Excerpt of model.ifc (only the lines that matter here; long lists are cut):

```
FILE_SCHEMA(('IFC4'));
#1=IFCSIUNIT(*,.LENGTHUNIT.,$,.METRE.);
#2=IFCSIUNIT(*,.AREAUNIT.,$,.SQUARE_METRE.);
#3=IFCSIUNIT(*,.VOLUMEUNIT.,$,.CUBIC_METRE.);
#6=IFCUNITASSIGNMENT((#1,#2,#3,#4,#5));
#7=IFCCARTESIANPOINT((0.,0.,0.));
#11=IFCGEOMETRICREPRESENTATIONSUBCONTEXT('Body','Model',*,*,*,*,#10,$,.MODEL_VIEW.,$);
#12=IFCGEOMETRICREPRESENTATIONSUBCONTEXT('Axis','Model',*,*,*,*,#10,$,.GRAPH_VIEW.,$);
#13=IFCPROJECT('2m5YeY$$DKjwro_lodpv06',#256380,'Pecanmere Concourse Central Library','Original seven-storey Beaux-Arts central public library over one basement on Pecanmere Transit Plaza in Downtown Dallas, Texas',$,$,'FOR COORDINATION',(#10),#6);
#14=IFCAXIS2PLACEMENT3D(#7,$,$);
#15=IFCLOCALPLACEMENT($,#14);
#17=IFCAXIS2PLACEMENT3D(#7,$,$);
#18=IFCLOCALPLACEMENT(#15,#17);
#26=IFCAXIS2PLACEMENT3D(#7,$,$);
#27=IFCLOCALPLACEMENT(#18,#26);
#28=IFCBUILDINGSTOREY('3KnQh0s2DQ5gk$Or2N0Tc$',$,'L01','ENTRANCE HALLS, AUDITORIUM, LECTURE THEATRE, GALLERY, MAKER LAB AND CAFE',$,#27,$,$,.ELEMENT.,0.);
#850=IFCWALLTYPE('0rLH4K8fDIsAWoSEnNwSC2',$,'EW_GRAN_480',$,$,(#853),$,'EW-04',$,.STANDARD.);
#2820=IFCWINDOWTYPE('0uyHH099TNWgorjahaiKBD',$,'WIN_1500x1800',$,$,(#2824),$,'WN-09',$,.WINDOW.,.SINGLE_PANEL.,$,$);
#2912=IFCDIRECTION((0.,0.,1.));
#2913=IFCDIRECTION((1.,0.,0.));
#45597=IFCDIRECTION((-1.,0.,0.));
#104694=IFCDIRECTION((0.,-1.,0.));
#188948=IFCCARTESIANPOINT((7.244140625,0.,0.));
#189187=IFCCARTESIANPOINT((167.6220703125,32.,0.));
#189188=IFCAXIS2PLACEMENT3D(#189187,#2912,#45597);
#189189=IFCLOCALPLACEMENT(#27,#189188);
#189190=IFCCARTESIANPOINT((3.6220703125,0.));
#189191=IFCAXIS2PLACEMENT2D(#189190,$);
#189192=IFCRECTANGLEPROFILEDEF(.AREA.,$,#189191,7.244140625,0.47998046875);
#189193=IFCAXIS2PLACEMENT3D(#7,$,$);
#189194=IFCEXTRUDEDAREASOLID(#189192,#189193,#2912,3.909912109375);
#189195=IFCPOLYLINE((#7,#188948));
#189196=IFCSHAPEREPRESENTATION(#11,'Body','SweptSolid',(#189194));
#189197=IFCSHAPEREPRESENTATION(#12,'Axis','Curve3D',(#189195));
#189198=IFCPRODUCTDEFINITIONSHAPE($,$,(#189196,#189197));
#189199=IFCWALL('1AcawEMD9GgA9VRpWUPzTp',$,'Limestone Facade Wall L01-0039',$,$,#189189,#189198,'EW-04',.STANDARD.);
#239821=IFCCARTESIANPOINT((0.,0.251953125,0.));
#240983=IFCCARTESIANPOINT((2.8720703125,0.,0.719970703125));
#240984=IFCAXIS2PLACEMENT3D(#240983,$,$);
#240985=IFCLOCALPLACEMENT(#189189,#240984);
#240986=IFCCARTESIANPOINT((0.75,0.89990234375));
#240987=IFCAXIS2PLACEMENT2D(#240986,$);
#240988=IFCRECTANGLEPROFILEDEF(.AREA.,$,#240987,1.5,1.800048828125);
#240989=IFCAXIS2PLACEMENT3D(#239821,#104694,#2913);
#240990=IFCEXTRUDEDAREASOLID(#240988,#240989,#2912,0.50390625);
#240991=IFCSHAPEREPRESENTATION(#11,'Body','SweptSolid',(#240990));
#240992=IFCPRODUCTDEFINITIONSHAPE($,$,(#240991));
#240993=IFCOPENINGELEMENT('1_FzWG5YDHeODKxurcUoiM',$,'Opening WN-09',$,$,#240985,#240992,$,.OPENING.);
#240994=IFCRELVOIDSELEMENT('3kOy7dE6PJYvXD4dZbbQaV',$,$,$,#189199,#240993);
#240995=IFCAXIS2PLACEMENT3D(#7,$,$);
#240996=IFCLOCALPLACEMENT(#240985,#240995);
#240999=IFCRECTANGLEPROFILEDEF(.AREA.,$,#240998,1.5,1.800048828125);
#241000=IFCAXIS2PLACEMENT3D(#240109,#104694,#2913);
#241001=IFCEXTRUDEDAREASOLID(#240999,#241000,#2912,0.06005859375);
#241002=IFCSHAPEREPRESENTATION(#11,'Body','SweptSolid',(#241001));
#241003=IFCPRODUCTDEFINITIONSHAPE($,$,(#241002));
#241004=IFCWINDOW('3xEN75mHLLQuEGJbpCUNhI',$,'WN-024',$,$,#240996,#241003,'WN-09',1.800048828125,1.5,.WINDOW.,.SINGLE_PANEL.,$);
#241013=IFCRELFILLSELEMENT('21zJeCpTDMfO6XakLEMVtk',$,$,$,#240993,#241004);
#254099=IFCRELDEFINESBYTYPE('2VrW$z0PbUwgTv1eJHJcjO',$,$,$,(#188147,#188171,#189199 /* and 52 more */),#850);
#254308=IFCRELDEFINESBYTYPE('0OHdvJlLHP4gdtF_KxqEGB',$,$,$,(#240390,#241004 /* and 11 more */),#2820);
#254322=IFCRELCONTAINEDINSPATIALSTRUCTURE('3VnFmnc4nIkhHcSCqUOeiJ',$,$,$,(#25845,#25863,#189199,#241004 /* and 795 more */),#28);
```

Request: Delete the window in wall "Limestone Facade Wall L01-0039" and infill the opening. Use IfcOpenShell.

```python
import ifcopenshell
import ifcopenshell.api.feature
import ifcopenshell.api.root
import ifcopenshell.geom
import ifcopenshell.util.shape

model = ifcopenshell.open("model.ifc")
settings = ifcopenshell.geom.settings()


def volume(element):
    """Net volume in cubic metres, openings subtracted."""
    shape = ifcopenshell.geom.create_shape(settings, element)
    return ifcopenshell.util.shape.get_volume(shape.geometry)


window = model.by_guid("3xEN75mHLLQuEGJbpCUNhI")
opening = window.FillsVoids[0].RelatingOpeningElement
wall = opening.VoidsElements[0].RelatingBuildingElement
before = volume(wall)

ifcopenshell.api.root.remove_product(model, product=window)
ifcopenshell.api.feature.remove_feature(model, feature=opening)

after = volume(wall)

print(f"wall volume {before:.3f} -> {after:.3f} m3")

model.write("model-out.ifc")
```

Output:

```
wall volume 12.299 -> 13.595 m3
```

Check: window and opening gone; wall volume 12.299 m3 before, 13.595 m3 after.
